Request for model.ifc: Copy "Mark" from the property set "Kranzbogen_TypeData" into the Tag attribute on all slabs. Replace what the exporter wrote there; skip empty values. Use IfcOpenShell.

First a look at what the model holds.

```python
import ifcopenshell
import ifcopenshell.util.element

model = ifcopenshell.open("model.ifc")
print(model.schema)
slabs = model.by_type("IfcSlab")
print(len(slabs), "slabs")
for e in slabs[:8]:
    source = ifcopenshell.util.element.get_pset(e, "Kranzbogen_TypeData", "Mark")
    target = e.Tag
    print(e.id(), repr(source), repr(target), sep=" | ")
```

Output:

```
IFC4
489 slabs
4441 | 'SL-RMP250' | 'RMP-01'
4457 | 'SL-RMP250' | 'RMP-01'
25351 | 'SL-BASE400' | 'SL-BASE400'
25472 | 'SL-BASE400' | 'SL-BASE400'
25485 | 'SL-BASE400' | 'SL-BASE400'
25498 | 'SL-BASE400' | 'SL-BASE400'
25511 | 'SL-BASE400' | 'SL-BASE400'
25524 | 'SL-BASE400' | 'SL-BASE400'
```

```python
import ifcopenshell
import ifcopenshell.util.element

model = ifcopenshell.open("model.ifc")

count = 0
for e in model.by_type("IfcSlab"):
    value = ifcopenshell.util.element.get_pset(e, "Kranzbogen_TypeData", "Mark")
    current = e.Tag
    if not value or not value.strip() or current == value:
        continue
    e.Tag = value
    count += 1

print(count, "slabs updated")

model.write("model-out.ifc")
```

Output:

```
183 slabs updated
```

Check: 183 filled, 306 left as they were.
